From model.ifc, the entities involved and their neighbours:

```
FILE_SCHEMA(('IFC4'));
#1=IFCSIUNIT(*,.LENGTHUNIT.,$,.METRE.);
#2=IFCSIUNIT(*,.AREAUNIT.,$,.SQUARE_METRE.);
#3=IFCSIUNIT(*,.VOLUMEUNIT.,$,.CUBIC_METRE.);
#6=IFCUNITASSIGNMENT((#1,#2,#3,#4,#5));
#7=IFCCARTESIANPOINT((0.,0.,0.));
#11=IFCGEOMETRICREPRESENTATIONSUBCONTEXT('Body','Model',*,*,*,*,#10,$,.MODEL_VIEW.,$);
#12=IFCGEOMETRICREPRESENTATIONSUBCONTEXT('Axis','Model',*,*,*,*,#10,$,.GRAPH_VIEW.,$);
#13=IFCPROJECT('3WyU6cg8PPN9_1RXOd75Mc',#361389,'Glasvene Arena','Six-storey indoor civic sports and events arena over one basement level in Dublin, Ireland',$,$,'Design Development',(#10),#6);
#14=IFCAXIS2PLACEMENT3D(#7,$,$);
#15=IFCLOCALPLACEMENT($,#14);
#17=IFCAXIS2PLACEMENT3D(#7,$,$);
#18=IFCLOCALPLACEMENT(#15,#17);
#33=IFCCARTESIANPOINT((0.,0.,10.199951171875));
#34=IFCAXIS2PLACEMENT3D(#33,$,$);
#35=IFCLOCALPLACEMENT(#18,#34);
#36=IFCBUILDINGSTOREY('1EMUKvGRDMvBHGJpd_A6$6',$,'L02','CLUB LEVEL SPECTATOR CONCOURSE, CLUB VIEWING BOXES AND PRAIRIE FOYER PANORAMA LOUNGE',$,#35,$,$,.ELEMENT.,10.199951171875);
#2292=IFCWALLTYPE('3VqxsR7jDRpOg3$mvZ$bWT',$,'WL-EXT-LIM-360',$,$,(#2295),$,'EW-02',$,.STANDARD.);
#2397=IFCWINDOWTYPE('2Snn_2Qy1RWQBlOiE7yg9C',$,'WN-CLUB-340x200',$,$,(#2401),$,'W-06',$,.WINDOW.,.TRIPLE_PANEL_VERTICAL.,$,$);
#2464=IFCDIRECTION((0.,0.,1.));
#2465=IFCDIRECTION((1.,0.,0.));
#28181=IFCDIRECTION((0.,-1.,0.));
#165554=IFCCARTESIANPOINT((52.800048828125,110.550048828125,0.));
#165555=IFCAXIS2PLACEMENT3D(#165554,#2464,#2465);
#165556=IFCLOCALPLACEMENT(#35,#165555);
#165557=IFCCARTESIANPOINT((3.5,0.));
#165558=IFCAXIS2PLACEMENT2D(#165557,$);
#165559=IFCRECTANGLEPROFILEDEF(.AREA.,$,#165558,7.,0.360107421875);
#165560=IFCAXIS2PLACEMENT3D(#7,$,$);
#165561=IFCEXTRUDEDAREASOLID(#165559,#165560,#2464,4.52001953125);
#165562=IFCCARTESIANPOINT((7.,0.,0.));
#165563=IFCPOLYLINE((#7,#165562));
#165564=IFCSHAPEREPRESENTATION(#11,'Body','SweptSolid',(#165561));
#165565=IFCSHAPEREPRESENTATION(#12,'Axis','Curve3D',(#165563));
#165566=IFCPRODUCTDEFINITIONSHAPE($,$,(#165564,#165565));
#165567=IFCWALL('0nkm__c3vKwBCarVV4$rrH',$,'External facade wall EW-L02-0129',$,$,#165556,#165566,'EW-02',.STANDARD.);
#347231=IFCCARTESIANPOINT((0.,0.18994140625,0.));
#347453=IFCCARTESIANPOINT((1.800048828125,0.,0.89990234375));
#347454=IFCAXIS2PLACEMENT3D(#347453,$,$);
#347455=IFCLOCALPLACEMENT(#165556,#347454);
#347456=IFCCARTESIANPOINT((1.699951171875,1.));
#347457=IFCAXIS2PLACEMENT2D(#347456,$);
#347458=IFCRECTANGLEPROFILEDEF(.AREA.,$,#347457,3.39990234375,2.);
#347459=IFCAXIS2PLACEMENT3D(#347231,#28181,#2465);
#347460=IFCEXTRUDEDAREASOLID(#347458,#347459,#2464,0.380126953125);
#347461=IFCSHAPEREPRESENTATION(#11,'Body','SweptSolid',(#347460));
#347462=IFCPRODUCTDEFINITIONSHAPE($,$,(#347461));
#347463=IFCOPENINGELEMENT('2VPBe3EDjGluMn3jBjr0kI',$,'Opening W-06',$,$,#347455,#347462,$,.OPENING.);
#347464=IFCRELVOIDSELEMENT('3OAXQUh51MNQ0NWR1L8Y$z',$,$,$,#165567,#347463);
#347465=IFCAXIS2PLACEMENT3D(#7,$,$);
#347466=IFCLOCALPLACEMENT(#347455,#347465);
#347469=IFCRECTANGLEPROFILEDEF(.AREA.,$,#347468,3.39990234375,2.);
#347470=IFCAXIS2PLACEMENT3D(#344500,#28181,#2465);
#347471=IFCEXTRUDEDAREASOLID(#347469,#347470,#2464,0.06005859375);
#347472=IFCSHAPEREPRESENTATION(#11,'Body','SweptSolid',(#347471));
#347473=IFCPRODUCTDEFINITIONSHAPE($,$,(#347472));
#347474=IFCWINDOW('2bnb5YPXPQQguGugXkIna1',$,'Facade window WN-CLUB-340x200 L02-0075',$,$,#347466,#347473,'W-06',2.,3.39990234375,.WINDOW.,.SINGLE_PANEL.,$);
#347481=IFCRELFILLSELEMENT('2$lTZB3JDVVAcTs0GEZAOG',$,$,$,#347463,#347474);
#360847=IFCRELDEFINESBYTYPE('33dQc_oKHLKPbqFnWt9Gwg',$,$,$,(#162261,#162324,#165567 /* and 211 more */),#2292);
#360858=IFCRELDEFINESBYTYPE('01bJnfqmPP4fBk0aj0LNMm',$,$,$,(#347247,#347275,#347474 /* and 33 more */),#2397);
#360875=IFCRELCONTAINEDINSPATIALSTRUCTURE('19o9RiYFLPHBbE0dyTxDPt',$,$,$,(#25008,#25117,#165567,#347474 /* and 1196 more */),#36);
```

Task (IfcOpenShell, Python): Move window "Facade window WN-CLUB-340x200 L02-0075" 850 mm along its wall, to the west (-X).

```python
import ifcopenshell
import ifcopenshell.api.geometry
import ifcopenshell.util.placement
import ifcopenshell.util.unit

model = ifcopenshell.open("model.ifc")
unit_scale = ifcopenshell.util.unit.calculate_unit_scale(model)

window = model.by_guid("2bnb5YPXPQQguGugXkIna1")
opening = window.FillsVoids[0].RelatingOpeningElement
wall = opening.VoidsElements[0].RelatingBuildingElement

wall_matrix = ifcopenshell.util.placement.get_local_placement(wall.ObjectPlacement)
shift = wall_matrix[:3, 0] * -0.85 / unit_scale
before = ifcopenshell.util.placement.get_local_placement(window.ObjectPlacement)[:3, 3].copy()

# The window is placed relative to its opening, so it follows when the opening moves.
matrix = ifcopenshell.util.placement.get_local_placement(opening.ObjectPlacement)
matrix[:3, 3] += shift
ifcopenshell.api.geometry.edit_object_placement(
    model, product=opening, matrix=matrix, is_si=False, should_transform_children=True
)

after = ifcopenshell.util.placement.get_local_placement(window.ObjectPlacement)[:3, 3]
print("window moved by", (after - before).round(3) + 0.0)

model.write("model_edited.ifc")
```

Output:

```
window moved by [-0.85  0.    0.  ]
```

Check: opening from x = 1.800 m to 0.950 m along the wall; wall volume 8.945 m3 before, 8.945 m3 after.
